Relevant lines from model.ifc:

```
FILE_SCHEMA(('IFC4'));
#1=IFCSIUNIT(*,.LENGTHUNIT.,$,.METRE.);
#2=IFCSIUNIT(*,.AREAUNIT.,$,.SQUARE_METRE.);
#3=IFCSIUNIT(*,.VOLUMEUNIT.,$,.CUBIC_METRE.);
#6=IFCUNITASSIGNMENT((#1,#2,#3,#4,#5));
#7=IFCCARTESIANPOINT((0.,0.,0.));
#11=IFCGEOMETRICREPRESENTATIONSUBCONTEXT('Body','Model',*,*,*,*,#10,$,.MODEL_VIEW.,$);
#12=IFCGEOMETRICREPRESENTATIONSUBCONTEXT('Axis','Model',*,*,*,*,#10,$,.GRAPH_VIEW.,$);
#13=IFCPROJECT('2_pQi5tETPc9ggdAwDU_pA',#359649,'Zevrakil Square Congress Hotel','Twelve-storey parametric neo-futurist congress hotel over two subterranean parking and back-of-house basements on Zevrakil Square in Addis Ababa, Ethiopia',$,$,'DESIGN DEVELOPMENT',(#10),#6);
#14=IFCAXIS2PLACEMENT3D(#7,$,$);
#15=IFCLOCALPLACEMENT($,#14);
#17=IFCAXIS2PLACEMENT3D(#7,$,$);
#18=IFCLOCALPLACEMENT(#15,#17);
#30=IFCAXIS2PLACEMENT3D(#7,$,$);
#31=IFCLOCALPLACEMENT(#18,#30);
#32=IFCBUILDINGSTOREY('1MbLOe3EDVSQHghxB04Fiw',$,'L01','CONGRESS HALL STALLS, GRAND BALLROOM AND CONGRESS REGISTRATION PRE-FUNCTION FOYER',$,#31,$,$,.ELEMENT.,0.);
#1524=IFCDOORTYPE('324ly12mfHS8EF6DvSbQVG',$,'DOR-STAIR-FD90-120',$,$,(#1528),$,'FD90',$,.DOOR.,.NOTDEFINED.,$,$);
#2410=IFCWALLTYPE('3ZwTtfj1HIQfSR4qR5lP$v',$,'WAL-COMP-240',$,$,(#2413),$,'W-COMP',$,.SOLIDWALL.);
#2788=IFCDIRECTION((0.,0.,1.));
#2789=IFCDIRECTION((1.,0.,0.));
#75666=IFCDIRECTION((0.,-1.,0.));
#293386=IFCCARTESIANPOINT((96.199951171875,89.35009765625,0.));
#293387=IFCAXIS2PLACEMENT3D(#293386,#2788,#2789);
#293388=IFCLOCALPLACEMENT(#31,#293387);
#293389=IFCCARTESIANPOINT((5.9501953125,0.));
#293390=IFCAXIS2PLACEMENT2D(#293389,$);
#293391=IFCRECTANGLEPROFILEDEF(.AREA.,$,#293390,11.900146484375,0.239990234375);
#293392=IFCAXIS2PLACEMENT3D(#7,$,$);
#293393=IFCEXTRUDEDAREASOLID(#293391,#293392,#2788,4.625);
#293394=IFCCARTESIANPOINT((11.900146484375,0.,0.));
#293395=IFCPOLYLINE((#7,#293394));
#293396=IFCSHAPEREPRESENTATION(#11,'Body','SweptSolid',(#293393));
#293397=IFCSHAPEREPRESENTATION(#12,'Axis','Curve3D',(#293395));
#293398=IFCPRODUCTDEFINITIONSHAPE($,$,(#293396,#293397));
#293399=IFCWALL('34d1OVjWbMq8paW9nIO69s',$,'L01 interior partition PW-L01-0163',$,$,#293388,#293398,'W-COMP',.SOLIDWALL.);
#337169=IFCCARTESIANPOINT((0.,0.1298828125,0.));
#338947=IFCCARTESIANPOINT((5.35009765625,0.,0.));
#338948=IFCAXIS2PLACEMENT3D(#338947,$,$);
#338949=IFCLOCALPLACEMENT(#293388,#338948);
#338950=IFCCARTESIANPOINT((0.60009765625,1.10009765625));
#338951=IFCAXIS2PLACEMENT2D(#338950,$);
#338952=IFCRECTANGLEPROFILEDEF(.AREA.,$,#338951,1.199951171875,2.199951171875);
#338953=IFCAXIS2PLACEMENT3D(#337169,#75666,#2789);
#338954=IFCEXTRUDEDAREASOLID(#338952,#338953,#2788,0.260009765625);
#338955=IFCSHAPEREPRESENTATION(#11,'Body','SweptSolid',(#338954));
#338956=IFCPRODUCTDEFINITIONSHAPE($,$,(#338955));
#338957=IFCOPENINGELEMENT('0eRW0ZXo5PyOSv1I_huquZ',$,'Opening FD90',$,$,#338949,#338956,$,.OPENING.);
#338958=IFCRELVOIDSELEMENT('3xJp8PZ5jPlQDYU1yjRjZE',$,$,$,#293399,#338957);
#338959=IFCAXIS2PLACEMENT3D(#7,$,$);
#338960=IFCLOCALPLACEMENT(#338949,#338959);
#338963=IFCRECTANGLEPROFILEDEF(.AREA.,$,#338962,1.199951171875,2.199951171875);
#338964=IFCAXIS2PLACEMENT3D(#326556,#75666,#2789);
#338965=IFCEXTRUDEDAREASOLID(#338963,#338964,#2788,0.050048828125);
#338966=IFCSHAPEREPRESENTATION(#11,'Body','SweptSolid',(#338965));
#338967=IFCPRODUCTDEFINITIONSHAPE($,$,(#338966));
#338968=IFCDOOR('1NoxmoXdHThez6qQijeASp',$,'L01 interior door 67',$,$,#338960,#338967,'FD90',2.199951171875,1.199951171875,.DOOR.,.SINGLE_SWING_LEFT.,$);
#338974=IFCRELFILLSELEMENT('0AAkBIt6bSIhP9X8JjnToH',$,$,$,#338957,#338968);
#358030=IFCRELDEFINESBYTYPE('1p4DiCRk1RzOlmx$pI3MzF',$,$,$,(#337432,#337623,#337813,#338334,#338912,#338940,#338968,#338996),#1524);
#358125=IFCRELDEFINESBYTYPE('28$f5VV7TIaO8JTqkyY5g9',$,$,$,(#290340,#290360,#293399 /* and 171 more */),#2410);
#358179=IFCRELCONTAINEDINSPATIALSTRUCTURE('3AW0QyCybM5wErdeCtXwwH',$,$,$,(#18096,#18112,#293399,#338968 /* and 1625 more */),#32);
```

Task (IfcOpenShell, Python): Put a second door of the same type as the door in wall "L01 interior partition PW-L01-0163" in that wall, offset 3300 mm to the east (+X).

```python
import ifcopenshell
import ifcopenshell.api.feature
import ifcopenshell.api.geometry
import ifcopenshell.api.root
import ifcopenshell.geom
import ifcopenshell.util.element
import ifcopenshell.util.placement
import ifcopenshell.util.shape

model = ifcopenshell.open("model.ifc")
settings = ifcopenshell.geom.settings()


def volume(element):
    """Net volume in cubic metres, openings subtracted."""
    shape = ifcopenshell.geom.create_shape(settings, element)
    return ifcopenshell.util.shape.get_volume(shape.geometry)


door = model.by_id(338968)
opening = door.FillsVoids[0].RelatingOpeningElement
wall = opening.VoidsElements[0].RelatingBuildingElement
before = volume(wall)
shift = ifcopenshell.util.placement.get_local_placement(wall.ObjectPlacement)[:3, 0] * 3.3

# copy_class copies the void relationship, type, container and properties, but no geometry.
new_opening = ifcopenshell.api.root.copy_class(model, product=opening)
new_opening.Representation = ifcopenshell.util.element.copy_deep(
    model, opening.Representation, exclude=["IfcGeometricRepresentationContext", "IfcRepresentationMap"]
)
new_door = ifcopenshell.api.root.copy_class(model, product=door)
new_door.Representation = ifcopenshell.util.element.copy_deep(
    model, door.Representation, exclude=["IfcGeometricRepresentationContext", "IfcRepresentationMap"]
)
new_door.Tag = None
ifcopenshell.api.feature.add_filling(model, opening=new_opening, element=new_door)

for old, new in ((opening, new_opening), (door, new_door)):
    matrix = ifcopenshell.util.placement.get_local_placement(old.ObjectPlacement)
    matrix[:3, 3] += shift
    ifcopenshell.api.geometry.edit_object_placement(model, product=new, matrix=matrix, is_si=False)

after = volume(wall)

print(f"wall volume {before:.3f} -> {after:.3f} m3")

model.write("model_edited.ifc")
```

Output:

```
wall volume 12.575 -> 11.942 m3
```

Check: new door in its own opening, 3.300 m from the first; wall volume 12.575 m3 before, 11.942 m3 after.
